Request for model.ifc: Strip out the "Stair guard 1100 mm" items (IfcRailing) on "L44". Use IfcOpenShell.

First a look at what the model holds.

```python
import ifcopenshell
import ifcopenshell.util.element

model = ifcopenshell.open("model.ifc")
print(model.schema)
storey = next(s for s in model.by_type("IfcBuildingStorey") if s.Name == "L44")
railings = [e for e in ifcopenshell.util.element.get_decomposition(storey) if e.is_a("IfcRailing")]
seen = {}
for e in railings:
    element_type = ifcopenshell.util.element.get_type(e)
    name = element_type.Name if element_type not in (None, e) else None
    seen[name] = seen.get(name, 0) + 1
for name, count in sorted(seen.items(), key=str):
    print(count, "x", name)
```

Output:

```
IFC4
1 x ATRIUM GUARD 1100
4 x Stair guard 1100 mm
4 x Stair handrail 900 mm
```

```python
import ifcopenshell
import ifcopenshell.api.root
import ifcopenshell.util.element

model = ifcopenshell.open("model.ifc")

storey = next(s for s in model.by_type("IfcBuildingStorey") if s.Name == "L44")
railings = [e for e in ifcopenshell.util.element.get_decomposition(storey) if e.is_a("IfcRailing")]
targets = [e for e in railings if (t := ifcopenshell.util.element.get_type(e)) not in (None, e) and t.Name == "Stair guard 1100 mm"]

for e in targets:
    ifcopenshell.api.root.remove_product(model, product=e)
print(len(targets), "removed")

model.write("model_rev.ifc")
```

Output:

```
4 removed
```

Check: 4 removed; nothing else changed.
